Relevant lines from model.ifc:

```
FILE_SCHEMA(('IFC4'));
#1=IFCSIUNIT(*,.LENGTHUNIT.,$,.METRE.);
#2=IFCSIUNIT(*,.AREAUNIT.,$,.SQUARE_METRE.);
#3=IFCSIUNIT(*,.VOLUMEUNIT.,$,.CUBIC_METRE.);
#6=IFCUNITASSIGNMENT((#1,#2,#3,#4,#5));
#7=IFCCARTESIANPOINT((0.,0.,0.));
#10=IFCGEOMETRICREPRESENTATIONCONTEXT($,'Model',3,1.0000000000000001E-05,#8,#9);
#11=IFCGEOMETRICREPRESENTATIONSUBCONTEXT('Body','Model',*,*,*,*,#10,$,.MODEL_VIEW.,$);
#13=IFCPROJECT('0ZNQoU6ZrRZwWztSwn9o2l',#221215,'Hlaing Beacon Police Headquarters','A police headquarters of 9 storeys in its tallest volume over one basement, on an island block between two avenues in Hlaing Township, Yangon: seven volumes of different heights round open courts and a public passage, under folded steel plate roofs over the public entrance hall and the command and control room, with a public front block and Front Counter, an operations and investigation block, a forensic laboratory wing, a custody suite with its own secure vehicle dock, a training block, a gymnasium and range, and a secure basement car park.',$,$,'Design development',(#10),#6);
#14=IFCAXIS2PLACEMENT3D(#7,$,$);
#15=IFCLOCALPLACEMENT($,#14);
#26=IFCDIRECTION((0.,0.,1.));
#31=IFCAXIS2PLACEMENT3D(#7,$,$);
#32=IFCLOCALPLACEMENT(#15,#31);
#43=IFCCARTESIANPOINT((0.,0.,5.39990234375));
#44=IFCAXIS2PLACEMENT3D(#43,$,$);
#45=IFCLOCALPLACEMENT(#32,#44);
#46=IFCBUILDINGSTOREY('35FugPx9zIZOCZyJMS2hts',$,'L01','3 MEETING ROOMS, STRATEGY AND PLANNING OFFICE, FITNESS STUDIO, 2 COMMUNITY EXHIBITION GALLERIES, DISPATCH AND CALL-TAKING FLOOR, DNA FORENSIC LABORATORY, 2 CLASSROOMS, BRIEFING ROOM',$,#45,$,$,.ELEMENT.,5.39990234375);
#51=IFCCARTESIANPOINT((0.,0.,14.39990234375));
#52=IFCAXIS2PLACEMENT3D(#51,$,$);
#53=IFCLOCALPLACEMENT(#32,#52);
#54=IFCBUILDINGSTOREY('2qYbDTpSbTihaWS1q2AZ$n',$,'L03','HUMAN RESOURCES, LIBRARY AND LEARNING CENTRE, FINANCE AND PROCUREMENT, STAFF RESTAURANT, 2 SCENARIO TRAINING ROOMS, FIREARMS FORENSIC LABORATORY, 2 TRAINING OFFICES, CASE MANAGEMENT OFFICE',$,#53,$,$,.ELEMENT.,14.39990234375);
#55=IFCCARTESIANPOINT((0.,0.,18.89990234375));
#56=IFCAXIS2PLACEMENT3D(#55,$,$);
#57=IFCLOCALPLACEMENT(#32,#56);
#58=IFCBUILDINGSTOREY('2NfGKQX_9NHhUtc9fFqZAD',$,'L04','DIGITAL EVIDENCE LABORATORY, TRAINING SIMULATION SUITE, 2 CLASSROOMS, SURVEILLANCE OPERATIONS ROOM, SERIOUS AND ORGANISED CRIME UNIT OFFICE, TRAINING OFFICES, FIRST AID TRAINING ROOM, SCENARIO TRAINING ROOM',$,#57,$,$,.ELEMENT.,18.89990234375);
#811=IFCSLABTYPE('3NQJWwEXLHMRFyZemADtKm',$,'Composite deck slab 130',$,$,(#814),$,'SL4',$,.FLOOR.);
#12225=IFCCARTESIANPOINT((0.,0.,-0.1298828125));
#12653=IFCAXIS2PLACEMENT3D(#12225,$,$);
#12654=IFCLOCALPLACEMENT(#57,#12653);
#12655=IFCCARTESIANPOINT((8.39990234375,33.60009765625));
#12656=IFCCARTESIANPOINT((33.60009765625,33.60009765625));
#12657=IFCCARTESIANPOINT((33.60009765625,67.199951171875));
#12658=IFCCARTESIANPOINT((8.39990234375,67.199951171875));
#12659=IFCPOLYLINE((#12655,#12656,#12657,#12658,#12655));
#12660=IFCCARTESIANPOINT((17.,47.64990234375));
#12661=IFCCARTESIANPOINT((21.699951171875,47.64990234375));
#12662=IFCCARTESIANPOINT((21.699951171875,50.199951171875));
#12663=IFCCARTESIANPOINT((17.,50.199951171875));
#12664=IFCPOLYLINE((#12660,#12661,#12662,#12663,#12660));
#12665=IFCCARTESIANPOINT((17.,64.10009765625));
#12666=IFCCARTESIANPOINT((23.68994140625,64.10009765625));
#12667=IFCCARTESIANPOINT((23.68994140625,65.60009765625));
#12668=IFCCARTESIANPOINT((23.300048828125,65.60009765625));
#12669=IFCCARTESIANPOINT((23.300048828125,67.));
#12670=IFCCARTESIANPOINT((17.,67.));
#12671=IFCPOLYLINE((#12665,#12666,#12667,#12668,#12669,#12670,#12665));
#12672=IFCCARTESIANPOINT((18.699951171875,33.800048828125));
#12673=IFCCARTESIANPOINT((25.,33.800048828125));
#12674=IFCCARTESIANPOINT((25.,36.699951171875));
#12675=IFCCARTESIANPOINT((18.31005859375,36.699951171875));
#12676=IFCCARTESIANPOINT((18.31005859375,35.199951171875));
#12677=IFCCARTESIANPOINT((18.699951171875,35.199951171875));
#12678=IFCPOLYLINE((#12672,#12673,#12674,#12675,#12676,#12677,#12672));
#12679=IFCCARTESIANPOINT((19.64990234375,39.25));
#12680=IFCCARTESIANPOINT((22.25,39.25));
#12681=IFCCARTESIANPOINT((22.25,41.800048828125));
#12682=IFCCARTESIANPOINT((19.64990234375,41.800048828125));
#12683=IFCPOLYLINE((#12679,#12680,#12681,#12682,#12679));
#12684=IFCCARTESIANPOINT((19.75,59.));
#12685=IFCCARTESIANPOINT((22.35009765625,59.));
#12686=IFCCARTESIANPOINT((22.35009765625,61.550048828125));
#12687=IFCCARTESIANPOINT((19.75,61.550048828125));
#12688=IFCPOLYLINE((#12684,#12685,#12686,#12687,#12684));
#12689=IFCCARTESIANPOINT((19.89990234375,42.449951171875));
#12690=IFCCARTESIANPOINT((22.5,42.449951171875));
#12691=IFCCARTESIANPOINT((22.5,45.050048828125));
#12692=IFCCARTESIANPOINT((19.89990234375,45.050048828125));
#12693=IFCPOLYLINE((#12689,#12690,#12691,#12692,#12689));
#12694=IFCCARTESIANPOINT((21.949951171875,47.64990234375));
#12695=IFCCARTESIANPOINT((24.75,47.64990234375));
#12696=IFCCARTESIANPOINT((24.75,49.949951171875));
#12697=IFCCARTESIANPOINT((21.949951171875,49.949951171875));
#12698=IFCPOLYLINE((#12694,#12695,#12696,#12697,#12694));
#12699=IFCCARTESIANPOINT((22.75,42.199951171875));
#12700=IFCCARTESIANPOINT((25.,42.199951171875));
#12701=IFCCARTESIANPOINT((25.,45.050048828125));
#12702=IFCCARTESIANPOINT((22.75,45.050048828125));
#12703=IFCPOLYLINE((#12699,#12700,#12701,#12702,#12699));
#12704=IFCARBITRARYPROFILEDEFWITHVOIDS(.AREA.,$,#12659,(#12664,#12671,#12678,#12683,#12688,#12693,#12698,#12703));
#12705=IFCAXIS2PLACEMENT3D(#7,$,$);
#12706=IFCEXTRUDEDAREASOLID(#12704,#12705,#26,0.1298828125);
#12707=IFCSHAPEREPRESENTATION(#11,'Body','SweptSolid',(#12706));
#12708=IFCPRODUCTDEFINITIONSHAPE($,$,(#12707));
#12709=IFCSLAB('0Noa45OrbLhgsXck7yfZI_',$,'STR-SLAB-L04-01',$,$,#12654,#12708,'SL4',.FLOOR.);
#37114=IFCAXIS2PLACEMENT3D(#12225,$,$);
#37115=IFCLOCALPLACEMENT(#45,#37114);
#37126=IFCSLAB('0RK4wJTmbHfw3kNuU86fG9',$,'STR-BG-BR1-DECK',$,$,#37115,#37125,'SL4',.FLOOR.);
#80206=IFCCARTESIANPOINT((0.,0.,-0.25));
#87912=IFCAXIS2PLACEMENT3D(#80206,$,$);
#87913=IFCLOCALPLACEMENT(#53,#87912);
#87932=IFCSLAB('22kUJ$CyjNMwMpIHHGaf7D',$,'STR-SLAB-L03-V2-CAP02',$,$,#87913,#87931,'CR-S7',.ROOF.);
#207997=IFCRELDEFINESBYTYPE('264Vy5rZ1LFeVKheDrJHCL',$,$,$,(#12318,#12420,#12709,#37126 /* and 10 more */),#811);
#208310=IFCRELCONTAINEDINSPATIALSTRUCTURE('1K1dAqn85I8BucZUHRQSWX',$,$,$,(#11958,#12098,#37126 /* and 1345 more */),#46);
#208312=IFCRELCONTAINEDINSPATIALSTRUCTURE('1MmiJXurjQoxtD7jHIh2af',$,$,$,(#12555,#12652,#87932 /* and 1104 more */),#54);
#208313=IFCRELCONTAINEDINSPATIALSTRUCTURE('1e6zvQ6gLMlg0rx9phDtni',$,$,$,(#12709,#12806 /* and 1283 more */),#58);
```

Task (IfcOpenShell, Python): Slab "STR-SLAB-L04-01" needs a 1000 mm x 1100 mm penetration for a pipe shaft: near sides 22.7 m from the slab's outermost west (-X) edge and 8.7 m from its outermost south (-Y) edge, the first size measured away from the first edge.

```python
import numpy as np
import ifcopenshell
import ifcopenshell.api.feature
import ifcopenshell.api.geometry
import ifcopenshell.api.root
import ifcopenshell.geom
import ifcopenshell.util.placement
import ifcopenshell.util.representation
import ifcopenshell.util.shape
import ifcopenshell.util.unit

model = ifcopenshell.open("model.ifc")
unit_scale = ifcopenshell.util.unit.calculate_unit_scale(model)
settings = ifcopenshell.geom.settings()


def volume(element):
    """Net volume in cubic metres, openings subtracted."""
    shape = ifcopenshell.geom.create_shape(settings, element)
    return ifcopenshell.util.shape.get_volume(shape.geometry)


slab = model.by_id(12709)
before = volume(slab)

# Extent in the slab's own axes, in metres. The edges named are its -X and -Y sides.
slab_shape = ifcopenshell.geom.create_shape(settings, slab)
vertices = ifcopenshell.util.shape.get_vertices(slab_shape.geometry)
x_min, y_min, bottom = vertices.min(axis=0)
top = vertices[:, 2].max()

opening = ifcopenshell.api.root.create_entity(model, ifc_class="IfcOpeningElement", name="Pipe shaft opening", predefined_type="OPENING")
context = ifcopenshell.util.representation.get_context(model, "Model", "Body", "MODEL_VIEW")
width, depth = 1, 1.1
outline = [(0.0, 0.0), (width, 0.0), (width, depth), (0.0, depth), (0.0, 0.0)]
# Overshoot both faces by 50 mm so the cut is clean.
shape = ifcopenshell.api.geometry.add_slab_representation(
    model, context=context, depth=top - bottom + 0.1, polyline=outline
)
ifcopenshell.api.geometry.assign_representation(model, product=opening, representation=shape)

matrix = ifcopenshell.util.placement.get_local_placement(slab.ObjectPlacement)
matrix[:, 3] = matrix @ np.append(np.array([x_min + 22.7, y_min + 8.7, bottom - 0.05]) / unit_scale, 1.0)
ifcopenshell.api.geometry.edit_object_placement(model, product=opening, matrix=matrix, is_si=False)
ifcopenshell.api.feature.add_feature(model, feature=opening, element=slab)

after = volume(slab)

print(f"slab volume {before:.3f} -> {after:.3f} m3")

model.write("model-out.ifc")
```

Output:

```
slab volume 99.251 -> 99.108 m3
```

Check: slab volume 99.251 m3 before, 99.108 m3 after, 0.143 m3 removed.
